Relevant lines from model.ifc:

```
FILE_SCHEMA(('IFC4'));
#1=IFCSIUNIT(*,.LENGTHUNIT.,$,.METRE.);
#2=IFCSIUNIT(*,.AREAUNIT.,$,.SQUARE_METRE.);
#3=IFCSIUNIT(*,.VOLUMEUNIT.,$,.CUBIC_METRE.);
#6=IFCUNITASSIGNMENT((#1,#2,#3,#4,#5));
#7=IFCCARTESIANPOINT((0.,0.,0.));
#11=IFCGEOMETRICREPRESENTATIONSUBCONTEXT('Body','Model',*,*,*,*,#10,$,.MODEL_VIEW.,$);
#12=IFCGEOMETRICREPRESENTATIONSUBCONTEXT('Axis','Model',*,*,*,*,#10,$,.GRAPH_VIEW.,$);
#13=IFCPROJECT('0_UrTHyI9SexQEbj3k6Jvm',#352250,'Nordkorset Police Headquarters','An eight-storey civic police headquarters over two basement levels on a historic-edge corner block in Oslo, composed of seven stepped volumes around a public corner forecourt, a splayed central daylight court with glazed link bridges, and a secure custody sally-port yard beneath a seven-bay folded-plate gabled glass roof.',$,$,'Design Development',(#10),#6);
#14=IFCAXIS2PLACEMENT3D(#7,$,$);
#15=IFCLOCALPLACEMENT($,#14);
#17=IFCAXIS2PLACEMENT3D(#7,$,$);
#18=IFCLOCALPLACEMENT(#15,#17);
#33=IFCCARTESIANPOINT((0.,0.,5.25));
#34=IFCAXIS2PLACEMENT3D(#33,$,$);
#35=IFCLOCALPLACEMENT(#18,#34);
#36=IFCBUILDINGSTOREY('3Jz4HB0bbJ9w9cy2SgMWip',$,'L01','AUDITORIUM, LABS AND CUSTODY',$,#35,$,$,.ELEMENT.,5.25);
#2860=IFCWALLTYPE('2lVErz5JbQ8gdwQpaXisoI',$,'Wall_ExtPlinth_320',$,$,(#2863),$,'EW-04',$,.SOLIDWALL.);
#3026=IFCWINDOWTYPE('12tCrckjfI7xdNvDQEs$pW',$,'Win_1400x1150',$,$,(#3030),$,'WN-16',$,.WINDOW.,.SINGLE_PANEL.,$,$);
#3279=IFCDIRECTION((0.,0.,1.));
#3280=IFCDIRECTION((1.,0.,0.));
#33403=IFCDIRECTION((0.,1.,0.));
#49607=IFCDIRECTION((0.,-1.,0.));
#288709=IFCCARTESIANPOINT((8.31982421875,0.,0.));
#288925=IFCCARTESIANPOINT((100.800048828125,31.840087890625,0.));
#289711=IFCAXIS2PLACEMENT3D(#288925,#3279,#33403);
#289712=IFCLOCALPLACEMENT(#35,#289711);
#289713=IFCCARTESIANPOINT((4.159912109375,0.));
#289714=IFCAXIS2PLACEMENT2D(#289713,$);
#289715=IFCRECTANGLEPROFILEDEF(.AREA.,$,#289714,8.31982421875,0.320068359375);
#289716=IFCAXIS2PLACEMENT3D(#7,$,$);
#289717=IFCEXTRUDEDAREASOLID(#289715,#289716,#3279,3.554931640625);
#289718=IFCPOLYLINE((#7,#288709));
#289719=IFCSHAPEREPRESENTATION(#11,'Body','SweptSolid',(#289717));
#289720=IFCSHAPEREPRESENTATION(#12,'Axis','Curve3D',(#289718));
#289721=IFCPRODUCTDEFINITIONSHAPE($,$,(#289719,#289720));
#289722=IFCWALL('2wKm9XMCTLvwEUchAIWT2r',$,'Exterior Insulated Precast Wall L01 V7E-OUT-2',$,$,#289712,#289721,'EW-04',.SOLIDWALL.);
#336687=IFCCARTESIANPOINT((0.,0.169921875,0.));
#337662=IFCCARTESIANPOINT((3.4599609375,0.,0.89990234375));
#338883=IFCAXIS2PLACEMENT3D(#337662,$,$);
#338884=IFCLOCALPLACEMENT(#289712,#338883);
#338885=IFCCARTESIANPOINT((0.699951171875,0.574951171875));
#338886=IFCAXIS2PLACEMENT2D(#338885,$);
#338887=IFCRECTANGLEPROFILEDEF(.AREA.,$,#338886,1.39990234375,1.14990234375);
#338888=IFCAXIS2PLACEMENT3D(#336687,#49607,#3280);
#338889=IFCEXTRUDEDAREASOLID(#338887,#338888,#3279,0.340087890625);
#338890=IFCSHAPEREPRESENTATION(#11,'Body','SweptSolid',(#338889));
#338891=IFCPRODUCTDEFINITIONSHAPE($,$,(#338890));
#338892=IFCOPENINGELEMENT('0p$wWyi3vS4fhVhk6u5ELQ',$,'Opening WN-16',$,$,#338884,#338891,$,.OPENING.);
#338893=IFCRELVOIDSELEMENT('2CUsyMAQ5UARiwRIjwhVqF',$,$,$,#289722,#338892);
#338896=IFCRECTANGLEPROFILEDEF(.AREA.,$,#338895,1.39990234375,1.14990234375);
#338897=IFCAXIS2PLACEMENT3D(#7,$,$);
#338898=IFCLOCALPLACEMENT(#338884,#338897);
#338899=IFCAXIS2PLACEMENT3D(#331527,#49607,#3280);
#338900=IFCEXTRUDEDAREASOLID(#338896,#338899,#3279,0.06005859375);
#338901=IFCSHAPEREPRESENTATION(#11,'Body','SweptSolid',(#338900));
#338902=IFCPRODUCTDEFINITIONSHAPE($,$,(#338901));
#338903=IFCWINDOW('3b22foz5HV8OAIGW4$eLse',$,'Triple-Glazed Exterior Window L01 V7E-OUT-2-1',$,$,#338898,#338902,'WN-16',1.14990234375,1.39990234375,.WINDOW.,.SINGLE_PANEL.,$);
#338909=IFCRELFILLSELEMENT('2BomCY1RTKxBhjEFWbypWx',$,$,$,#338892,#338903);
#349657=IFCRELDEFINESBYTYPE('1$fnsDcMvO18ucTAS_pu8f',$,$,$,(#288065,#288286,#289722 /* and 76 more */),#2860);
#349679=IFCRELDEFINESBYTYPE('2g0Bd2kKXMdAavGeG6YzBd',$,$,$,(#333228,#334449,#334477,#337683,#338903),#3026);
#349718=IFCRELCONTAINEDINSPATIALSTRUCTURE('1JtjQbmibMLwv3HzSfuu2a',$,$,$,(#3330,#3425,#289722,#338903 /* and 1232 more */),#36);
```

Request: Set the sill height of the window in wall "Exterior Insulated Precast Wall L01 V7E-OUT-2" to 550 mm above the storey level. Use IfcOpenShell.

```python
import numpy as np
import ifcopenshell
import ifcopenshell.api.geometry
import ifcopenshell.geom
import ifcopenshell.util.element
import ifcopenshell.util.placement
import ifcopenshell.util.shape
import ifcopenshell.util.unit

model = ifcopenshell.open("model.ifc")
unit_scale = ifcopenshell.util.unit.calculate_unit_scale(model)

window = model.by_guid("3b22foz5HV8OAIGW4$eLse")
opening = window.FillsVoids[0].RelatingOpeningElement
storey = ifcopenshell.util.element.get_container(window, ifc_class="IfcBuildingStorey")
level = ifcopenshell.util.placement.get_local_placement(storey.ObjectPlacement)[2, 3]

# The opening's origin need not be at the sill, so measure its lowest point.
shape = ifcopenshell.geom.create_shape(ifcopenshell.geom.settings(), opening)
bottom = ifcopenshell.util.shape.get_shape_bottom_elevation(shape, shape.geometry) / unit_scale
dz = level + 0.55 / unit_scale - bottom

shift = np.array([0.0, 0.0, dz])
# The window is placed relative to its opening, so it follows when the opening moves.
matrix = ifcopenshell.util.placement.get_local_placement(opening.ObjectPlacement)
matrix[:3, 3] += shift
ifcopenshell.api.geometry.edit_object_placement(
    model, product=opening, matrix=matrix, is_si=False, should_transform_children=True
)

print(f"moved by {dz * unit_scale:+.3f} m")

model.write("model_updated.ifc")
```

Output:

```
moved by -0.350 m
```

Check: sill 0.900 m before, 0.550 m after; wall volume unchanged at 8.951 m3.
